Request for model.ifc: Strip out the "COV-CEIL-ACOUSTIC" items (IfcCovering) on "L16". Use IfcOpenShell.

First a look at what the model holds.

```python
import ifcopenshell
import ifcopenshell.util.element

model = ifcopenshell.open("model.ifc")
print(model.schema)
storey = next(s for s in model.by_type("IfcBuildingStorey") if s.Name == "L16")
coverings = [e for e in ifcopenshell.util.element.get_decomposition(storey) if e.is_a("IfcCovering")]
seen = {}
for e in coverings:
    element_type = ifcopenshell.util.element.get_type(e)
    name = element_type.Name if element_type not in (None, e) else None
    seen[name] = seen.get(name, 0) + 1
for name, count in sorted(seen.items(), key=str):
    print(count, "x", name)
```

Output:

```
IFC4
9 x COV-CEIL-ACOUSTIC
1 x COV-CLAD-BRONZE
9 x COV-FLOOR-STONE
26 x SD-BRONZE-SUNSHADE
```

```python
import ifcopenshell
import ifcopenshell.api.root
import ifcopenshell.util.element

model = ifcopenshell.open("model.ifc")

storey = next(s for s in model.by_type("IfcBuildingStorey") if s.Name == "L16")
coverings = [e for e in ifcopenshell.util.element.get_decomposition(storey) if e.is_a("IfcCovering")]
targets = [e for e in coverings if (t := ifcopenshell.util.element.get_type(e)) not in (None, e) and t.Name == "COV-CEIL-ACOUSTIC"]

for e in targets:
    ifcopenshell.api.root.remove_product(model, product=e)
print(len(targets), "removed")

model.write("model-out.ifc")
```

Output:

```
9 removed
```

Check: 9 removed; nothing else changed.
